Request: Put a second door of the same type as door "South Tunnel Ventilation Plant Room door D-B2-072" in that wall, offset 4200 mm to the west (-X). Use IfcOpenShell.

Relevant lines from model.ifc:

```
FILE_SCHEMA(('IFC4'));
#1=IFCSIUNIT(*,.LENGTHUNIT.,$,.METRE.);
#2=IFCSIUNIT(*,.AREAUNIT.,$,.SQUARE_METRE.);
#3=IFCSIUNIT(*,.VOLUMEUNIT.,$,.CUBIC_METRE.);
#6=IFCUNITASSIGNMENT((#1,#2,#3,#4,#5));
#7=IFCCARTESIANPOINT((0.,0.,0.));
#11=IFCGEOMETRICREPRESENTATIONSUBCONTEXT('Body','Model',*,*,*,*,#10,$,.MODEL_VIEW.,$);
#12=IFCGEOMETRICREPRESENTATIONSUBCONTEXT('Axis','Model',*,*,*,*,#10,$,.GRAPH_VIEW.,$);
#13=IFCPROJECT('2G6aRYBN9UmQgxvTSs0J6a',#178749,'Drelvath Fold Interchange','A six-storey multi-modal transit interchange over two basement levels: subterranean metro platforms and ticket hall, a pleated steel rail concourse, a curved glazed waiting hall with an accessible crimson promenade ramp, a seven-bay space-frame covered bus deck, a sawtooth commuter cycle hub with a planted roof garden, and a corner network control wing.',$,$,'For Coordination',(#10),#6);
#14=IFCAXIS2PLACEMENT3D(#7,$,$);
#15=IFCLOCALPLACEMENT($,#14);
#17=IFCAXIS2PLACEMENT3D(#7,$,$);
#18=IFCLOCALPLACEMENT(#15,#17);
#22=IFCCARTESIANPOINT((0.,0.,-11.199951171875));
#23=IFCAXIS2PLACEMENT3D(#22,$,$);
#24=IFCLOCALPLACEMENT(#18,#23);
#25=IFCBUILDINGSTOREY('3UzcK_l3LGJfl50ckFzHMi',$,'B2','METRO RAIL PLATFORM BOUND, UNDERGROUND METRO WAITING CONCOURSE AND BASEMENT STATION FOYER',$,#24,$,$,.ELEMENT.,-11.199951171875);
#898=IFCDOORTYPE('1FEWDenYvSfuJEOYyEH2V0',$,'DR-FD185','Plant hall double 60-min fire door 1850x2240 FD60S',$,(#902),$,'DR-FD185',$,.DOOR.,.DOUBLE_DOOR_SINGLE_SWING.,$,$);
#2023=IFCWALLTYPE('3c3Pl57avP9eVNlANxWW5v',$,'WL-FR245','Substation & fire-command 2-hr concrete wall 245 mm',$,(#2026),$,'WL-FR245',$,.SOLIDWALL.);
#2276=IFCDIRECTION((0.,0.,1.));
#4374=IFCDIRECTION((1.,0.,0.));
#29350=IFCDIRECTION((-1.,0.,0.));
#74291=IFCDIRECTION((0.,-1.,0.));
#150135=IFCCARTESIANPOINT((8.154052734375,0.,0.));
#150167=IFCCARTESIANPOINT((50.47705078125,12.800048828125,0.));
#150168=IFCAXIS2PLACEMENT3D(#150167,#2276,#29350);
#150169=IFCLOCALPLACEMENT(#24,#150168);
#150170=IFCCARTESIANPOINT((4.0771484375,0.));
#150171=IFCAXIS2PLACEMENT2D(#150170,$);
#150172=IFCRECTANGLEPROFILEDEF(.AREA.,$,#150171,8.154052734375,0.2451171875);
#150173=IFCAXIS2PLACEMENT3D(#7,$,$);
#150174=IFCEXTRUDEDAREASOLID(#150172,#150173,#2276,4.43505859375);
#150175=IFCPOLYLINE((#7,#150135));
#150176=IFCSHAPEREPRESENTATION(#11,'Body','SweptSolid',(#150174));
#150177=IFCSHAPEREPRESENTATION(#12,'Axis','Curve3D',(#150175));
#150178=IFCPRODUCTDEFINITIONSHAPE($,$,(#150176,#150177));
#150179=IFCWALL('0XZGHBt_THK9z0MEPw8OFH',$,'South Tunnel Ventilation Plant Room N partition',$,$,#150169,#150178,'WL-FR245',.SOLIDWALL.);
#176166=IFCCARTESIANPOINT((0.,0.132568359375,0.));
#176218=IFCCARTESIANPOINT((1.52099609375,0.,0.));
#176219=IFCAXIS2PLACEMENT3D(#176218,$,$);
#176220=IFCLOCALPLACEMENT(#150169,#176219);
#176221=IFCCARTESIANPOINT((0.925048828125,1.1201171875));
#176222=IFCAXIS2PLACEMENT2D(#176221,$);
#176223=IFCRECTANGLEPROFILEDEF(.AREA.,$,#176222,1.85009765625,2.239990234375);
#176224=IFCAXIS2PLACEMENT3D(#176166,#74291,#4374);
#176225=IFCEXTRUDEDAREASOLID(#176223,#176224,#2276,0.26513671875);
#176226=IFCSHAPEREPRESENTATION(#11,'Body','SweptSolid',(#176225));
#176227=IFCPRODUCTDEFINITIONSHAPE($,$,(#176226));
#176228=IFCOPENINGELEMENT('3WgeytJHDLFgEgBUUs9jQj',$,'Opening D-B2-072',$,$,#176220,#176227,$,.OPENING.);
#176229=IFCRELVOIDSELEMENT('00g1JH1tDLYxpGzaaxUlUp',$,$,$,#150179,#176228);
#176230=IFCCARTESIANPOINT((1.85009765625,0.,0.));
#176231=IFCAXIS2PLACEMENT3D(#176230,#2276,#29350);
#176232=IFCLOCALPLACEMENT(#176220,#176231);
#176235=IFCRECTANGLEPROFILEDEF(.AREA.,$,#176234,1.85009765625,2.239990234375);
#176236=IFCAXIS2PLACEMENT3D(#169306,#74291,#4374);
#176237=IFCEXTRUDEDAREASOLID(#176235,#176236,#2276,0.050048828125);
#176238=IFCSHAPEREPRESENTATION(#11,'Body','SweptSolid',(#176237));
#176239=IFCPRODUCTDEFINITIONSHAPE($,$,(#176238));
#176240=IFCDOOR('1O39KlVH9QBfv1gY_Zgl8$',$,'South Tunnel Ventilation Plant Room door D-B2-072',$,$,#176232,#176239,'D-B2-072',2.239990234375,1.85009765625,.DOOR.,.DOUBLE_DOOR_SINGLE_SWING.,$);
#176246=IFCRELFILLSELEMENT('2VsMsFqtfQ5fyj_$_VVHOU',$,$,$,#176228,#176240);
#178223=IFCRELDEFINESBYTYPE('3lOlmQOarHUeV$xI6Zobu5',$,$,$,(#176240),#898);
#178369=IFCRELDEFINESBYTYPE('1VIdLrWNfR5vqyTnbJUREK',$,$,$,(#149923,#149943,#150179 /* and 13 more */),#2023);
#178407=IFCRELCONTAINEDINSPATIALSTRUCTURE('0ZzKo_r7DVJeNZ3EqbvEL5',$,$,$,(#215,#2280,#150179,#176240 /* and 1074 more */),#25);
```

```python
import ifcopenshell
import ifcopenshell.api.feature
import ifcopenshell.api.geometry
import ifcopenshell.api.root
import ifcopenshell.geom
import ifcopenshell.util.element
import ifcopenshell.util.placement
import ifcopenshell.util.shape
import ifcopenshell.util.unit

model = ifcopenshell.open("model.ifc")
unit_scale = ifcopenshell.util.unit.calculate_unit_scale(model)
settings = ifcopenshell.geom.settings()


def volume(element):
    """Net volume in cubic metres, openings subtracted."""
    shape = ifcopenshell.geom.create_shape(settings, element)
    return ifcopenshell.util.shape.get_volume(shape.geometry)


door = model.by_guid("1O39KlVH9QBfv1gY_Zgl8$")
opening = door.FillsVoids[0].RelatingOpeningElement
wall = opening.VoidsElements[0].RelatingBuildingElement
before = volume(wall)
shift = ifcopenshell.util.placement.get_local_placement(wall.ObjectPlacement)[:3, 0] * 4.2 / unit_scale

# copy_class copies the void relationship, type, container and properties, but no geometry.
new_opening = ifcopenshell.api.root.copy_class(model, product=opening)
new_opening.Representation = ifcopenshell.util.element.copy_deep(
    model, opening.Representation, exclude=["IfcGeometricRepresentationContext", "IfcRepresentationMap"]
)
new_door = ifcopenshell.api.root.copy_class(model, product=door)
new_door.Representation = ifcopenshell.util.element.copy_deep(
    model, door.Representation, exclude=["IfcGeometricRepresentationContext", "IfcRepresentationMap"]
)
new_door.Tag = None
ifcopenshell.api.feature.add_filling(model, opening=new_opening, element=new_door)

for old, new in ((opening, new_opening), (door, new_door)):
    matrix = ifcopenshell.util.placement.get_local_placement(old.ObjectPlacement)
    matrix[:3, 3] += shift
    ifcopenshell.api.geometry.edit_object_placement(model, product=new, matrix=matrix, is_si=False)

after = volume(wall)

print(f"wall volume {before:.3f} -> {after:.3f} m3")

model.write("model-out.ifc")
```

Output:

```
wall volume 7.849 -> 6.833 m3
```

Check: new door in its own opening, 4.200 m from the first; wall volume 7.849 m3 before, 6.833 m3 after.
